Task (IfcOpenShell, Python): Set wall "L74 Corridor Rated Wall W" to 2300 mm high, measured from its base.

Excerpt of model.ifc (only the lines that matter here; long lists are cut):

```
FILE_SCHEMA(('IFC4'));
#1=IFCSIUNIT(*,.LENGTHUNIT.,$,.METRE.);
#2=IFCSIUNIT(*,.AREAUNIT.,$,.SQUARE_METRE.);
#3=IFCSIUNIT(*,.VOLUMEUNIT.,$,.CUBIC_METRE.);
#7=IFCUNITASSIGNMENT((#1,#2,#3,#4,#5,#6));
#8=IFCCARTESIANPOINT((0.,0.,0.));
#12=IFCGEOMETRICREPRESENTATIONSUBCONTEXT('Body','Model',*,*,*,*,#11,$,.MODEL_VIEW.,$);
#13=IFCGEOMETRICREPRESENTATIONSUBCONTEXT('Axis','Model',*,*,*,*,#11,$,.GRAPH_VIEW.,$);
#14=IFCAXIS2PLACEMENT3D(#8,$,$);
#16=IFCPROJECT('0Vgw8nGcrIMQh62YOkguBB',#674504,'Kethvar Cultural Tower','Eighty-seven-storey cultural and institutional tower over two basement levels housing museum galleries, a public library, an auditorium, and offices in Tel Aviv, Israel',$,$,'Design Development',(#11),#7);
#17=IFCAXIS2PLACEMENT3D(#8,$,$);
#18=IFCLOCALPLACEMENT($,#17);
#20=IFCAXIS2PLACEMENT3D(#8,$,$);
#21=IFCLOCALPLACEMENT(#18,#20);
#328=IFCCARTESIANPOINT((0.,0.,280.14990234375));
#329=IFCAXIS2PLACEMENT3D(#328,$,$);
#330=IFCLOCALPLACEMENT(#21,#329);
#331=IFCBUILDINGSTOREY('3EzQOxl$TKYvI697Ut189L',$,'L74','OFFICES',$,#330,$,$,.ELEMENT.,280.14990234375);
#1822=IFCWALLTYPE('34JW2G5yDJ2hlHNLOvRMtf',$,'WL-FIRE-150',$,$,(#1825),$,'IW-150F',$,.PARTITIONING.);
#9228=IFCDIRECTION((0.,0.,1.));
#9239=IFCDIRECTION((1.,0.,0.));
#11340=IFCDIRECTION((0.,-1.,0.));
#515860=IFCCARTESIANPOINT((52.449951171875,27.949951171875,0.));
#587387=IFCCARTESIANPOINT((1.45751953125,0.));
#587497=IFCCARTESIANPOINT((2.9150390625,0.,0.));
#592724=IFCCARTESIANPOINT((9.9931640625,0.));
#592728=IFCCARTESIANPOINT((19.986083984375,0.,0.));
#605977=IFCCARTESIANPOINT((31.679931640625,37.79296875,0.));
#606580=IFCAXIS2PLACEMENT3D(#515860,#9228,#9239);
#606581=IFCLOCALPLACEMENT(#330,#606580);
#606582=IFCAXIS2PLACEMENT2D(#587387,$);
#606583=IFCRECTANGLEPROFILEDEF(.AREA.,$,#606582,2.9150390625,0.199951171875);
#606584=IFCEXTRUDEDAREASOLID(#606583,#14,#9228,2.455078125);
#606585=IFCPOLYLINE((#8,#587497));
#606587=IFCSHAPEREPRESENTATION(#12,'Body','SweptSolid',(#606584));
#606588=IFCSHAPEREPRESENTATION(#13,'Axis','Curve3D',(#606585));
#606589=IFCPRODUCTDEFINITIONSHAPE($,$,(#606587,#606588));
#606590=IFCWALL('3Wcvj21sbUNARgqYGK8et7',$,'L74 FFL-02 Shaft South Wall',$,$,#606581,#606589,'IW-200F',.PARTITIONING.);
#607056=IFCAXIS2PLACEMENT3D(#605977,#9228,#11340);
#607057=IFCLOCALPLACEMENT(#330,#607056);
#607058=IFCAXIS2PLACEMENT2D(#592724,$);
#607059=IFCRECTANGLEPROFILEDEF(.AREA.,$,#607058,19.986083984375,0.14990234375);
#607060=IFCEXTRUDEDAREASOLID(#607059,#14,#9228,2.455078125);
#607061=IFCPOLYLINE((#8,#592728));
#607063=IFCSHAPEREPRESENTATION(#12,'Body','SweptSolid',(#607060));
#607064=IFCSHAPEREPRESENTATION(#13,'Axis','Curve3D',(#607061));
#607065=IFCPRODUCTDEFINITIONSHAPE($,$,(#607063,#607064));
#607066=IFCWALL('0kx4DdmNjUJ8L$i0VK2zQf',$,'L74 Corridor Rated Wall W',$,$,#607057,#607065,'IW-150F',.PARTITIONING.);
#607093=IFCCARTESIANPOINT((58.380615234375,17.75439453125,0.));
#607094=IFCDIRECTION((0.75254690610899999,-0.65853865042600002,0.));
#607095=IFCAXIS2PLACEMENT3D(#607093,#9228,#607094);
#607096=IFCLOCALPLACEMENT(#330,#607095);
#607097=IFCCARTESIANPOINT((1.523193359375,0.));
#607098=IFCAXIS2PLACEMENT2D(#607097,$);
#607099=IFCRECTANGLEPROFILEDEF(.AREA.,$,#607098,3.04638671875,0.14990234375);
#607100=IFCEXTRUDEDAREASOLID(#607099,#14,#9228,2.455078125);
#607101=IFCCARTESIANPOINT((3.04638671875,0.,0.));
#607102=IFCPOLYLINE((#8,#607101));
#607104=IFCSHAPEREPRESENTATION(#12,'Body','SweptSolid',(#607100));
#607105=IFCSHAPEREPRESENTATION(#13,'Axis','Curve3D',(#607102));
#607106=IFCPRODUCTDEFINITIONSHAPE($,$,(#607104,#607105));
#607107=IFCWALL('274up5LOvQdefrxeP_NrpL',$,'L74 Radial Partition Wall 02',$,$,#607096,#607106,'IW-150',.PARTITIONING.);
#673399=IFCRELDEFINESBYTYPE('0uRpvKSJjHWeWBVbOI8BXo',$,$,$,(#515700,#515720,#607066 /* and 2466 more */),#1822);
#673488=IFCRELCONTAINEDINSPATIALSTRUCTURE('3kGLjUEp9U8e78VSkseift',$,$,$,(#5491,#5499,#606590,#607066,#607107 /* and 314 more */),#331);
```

```python
import ifcopenshell
import ifcopenshell.geom
import ifcopenshell.util.representation
import ifcopenshell.util.shape
import ifcopenshell.util.unit

model = ifcopenshell.open("model.ifc")
unit_scale = ifcopenshell.util.unit.calculate_unit_scale(model)
settings = ifcopenshell.geom.settings()


def volume(element):
    """Net volume in cubic metres, openings subtracted."""
    shape = ifcopenshell.geom.create_shape(settings, element)
    return ifcopenshell.util.shape.get_volume(shape.geometry)


wall = model.by_id(607066)
before = volume(wall)

body = ifcopenshell.util.representation.get_representation(wall, "Model", "Body")
solid = body.Items[0]
old_height = solid.Depth
solid.Depth = 2.3 / unit_scale
after = volume(wall)

print(f"height {old_height:g} -> {solid.Depth:g}, volume {before:.3f} -> {after:.3f} m3")

model.write("model-out.ifc")
```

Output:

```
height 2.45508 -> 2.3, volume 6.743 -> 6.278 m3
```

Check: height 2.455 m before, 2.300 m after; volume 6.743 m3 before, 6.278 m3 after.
